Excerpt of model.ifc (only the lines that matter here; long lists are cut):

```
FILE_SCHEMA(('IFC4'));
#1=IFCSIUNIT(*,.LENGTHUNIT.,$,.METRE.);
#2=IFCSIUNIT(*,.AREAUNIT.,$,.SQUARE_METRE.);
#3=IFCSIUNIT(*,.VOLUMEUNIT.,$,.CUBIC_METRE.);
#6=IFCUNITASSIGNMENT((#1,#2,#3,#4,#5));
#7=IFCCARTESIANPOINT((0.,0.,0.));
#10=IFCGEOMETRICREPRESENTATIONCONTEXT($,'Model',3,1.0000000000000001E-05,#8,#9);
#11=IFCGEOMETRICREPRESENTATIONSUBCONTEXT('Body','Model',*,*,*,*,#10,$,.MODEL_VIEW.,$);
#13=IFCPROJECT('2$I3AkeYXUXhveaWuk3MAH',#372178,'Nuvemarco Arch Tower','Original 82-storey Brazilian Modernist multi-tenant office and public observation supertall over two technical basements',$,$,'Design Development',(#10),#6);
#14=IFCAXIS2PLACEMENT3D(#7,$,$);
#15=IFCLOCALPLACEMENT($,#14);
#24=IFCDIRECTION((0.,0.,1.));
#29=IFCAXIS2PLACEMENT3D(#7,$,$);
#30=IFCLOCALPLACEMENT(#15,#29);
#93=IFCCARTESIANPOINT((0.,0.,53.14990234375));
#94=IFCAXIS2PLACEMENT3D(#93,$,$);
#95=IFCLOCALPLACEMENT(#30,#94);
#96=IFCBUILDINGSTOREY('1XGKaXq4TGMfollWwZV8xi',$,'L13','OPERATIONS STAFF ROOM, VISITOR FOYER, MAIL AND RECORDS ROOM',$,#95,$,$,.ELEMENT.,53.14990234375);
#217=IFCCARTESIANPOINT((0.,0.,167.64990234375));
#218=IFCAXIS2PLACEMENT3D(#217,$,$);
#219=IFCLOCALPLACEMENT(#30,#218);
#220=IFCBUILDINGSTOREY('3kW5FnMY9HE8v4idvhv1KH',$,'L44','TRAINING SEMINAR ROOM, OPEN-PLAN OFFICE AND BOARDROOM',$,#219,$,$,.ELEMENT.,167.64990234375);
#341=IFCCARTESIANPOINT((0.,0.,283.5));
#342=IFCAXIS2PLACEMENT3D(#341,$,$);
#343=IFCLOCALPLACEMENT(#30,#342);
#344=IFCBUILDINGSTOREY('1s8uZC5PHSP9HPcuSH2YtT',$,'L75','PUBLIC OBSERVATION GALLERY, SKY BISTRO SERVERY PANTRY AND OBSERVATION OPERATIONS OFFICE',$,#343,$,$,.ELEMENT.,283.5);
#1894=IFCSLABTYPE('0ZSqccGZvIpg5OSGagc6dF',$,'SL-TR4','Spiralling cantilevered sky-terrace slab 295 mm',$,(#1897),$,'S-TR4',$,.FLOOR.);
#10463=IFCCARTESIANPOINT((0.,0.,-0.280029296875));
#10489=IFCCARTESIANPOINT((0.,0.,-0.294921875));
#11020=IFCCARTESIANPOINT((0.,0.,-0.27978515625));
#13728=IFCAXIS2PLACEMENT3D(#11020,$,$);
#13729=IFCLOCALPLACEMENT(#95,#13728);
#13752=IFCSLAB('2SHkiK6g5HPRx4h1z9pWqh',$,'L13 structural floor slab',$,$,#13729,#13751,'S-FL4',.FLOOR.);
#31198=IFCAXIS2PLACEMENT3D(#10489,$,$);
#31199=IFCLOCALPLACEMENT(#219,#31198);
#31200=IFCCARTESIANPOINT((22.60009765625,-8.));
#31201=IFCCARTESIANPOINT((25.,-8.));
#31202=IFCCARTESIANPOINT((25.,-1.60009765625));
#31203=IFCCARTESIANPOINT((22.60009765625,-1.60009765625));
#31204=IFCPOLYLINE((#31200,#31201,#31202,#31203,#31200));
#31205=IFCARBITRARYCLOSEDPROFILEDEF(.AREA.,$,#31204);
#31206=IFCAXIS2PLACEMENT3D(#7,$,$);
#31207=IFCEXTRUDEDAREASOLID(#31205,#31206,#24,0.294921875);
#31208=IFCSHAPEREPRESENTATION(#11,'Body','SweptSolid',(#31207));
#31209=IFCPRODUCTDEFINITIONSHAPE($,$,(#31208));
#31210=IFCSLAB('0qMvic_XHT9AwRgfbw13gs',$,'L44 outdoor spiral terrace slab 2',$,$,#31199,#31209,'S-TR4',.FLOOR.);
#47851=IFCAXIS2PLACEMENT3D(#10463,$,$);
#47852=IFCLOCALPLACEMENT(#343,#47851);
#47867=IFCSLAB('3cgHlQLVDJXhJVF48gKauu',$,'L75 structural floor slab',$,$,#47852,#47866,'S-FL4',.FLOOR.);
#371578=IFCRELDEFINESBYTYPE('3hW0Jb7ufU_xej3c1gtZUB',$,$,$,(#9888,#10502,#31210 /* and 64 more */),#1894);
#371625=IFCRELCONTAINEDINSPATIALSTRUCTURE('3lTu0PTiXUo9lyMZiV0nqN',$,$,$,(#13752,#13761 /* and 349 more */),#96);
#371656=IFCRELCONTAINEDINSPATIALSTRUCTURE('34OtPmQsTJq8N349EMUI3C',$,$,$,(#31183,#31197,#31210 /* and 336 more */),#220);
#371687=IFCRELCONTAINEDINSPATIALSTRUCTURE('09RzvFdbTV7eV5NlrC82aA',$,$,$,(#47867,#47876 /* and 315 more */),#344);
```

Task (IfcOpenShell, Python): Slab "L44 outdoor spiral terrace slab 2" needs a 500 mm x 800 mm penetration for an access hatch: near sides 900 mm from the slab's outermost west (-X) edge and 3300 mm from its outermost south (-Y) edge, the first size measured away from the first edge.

```python
import numpy as np
import ifcopenshell
import ifcopenshell.api.feature
import ifcopenshell.api.geometry
import ifcopenshell.api.root
import ifcopenshell.geom
import ifcopenshell.util.placement
import ifcopenshell.util.representation
import ifcopenshell.util.shape
import ifcopenshell.util.unit

model = ifcopenshell.open("model.ifc")
unit_scale = ifcopenshell.util.unit.calculate_unit_scale(model)
settings = ifcopenshell.geom.settings()


def volume(element):
    """Net volume in cubic metres, openings subtracted."""
    shape = ifcopenshell.geom.create_shape(settings, element)
    return ifcopenshell.util.shape.get_volume(shape.geometry)


slab = model.by_guid("0qMvic_XHT9AwRgfbw13gs")
before = volume(slab)

# Extent in the slab's own axes, in metres. The edges named are its -X and -Y sides.
slab_shape = ifcopenshell.geom.create_shape(settings, slab)
vertices = ifcopenshell.util.shape.get_vertices(slab_shape.geometry)
x_min, y_min, bottom = vertices.min(axis=0)
top = vertices[:, 2].max()

opening = ifcopenshell.api.root.create_entity(model, ifc_class="IfcOpeningElement", name="Access hatch opening", predefined_type="OPENING")
context = ifcopenshell.util.representation.get_context(model, "Model", "Body", "MODEL_VIEW")
width, depth = 0.5, 0.8
outline = [(0.0, 0.0), (width, 0.0), (width, depth), (0.0, depth), (0.0, 0.0)]
# Overshoot both faces by 50 mm so the cut is clean.
shape = ifcopenshell.api.geometry.add_slab_representation(
    model, context=context, depth=top - bottom + 0.1, polyline=outline
)
ifcopenshell.api.geometry.assign_representation(model, product=opening, representation=shape)

matrix = ifcopenshell.util.placement.get_local_placement(slab.ObjectPlacement)
matrix[:, 3] = matrix @ np.append(np.array([x_min + 0.9, y_min + 3.3, bottom - 0.05]) / unit_scale, 1.0)
ifcopenshell.api.geometry.edit_object_placement(model, product=opening, matrix=matrix, is_si=False)
ifcopenshell.api.feature.add_feature(model, feature=opening, element=slab)

after = volume(slab)

print(f"slab volume {before:.3f} -> {after:.3f} m3")

model.write("model_v2.ifc")
```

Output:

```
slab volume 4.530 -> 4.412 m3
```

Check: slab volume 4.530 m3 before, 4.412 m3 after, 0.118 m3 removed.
